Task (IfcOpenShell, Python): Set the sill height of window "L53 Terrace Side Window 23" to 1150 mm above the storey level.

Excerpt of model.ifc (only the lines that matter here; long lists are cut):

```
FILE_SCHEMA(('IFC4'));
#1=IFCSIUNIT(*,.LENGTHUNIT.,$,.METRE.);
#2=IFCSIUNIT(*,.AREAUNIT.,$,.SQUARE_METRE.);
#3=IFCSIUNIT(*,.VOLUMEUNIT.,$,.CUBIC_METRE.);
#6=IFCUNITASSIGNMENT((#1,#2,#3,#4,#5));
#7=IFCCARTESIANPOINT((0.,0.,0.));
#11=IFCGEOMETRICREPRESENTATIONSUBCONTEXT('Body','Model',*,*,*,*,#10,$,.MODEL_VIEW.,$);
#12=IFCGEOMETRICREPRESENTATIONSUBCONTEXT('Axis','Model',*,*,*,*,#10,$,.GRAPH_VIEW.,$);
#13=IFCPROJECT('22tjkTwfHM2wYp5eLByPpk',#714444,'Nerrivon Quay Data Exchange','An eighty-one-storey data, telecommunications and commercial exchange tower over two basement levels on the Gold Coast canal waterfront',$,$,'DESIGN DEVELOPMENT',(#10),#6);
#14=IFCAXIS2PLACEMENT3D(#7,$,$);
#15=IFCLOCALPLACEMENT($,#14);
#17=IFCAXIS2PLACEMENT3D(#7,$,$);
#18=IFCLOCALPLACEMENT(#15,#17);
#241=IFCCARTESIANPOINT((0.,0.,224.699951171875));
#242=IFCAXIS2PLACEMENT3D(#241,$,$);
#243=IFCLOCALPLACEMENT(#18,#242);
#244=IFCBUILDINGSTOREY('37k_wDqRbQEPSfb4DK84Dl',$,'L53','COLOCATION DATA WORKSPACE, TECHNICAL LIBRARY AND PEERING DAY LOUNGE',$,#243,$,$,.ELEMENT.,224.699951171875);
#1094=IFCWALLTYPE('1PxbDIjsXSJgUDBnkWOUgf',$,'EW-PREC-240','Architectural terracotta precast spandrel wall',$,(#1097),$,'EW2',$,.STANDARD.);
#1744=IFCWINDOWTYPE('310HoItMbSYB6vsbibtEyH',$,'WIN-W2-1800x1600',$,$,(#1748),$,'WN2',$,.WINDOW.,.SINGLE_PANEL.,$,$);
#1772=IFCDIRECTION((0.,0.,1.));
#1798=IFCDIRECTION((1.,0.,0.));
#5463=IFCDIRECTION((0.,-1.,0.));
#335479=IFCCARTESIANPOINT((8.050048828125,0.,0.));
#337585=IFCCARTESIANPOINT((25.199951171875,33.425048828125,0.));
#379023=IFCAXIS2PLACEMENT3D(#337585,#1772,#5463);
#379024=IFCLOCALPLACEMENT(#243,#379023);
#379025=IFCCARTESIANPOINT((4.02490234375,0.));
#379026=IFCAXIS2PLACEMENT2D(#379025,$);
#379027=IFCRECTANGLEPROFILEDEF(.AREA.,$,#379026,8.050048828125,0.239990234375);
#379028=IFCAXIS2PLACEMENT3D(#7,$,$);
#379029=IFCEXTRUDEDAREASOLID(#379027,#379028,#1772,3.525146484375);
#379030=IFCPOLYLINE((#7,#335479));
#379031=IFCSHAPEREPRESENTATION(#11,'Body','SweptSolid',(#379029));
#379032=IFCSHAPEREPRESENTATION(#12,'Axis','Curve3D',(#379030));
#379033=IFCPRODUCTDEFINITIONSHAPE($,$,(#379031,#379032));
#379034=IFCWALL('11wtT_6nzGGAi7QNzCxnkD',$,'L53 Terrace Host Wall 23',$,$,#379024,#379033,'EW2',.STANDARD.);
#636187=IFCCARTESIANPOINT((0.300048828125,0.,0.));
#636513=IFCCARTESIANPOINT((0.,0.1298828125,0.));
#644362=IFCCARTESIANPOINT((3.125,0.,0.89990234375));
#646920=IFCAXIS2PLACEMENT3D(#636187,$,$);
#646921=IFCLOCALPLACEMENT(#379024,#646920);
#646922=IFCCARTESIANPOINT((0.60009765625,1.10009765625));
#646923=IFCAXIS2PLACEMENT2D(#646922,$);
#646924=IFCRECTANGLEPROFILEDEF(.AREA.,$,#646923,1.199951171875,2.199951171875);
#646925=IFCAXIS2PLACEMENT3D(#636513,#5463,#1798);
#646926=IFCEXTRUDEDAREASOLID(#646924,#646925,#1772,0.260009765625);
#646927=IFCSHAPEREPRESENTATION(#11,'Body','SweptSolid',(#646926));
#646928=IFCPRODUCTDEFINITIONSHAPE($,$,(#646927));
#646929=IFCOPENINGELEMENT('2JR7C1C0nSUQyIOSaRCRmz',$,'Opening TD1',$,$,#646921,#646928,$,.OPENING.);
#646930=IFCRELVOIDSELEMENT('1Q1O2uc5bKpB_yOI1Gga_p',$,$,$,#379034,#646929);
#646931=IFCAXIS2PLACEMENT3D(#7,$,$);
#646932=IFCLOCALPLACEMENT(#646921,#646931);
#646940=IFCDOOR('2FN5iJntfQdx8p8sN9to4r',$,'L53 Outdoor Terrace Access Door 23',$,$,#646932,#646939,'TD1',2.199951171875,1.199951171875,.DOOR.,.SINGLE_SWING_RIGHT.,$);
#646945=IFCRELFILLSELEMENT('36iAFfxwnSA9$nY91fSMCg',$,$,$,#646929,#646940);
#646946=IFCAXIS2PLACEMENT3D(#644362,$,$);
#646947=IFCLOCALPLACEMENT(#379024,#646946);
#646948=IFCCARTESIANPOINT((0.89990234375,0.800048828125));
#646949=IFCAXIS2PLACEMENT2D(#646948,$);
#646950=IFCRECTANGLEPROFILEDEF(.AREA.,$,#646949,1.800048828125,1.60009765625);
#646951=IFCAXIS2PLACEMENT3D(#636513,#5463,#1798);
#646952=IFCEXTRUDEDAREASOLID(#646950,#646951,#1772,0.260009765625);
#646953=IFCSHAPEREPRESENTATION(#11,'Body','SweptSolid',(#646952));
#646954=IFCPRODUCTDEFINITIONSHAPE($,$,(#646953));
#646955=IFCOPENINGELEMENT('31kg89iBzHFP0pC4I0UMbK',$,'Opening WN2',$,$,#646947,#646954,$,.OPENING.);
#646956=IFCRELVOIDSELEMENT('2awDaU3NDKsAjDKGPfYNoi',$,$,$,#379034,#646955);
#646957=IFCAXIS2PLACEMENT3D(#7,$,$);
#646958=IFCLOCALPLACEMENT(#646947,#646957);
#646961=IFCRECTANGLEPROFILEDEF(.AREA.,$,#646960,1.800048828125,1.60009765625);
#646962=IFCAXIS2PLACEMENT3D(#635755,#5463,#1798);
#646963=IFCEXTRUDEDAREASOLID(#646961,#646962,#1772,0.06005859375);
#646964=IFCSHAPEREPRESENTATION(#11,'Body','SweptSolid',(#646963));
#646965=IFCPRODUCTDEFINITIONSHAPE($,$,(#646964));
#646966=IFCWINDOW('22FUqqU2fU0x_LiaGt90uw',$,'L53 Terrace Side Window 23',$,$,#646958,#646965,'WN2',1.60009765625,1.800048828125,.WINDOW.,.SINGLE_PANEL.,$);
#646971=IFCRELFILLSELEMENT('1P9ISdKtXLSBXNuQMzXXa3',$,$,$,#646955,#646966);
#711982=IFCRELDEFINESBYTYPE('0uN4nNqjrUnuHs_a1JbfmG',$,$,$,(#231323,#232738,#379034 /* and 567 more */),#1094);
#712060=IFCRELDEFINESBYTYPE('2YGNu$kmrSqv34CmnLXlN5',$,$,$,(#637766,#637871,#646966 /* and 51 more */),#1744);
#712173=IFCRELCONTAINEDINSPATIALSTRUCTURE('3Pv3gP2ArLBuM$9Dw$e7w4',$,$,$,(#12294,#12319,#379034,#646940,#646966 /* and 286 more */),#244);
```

```python
import numpy as np
import ifcopenshell
import ifcopenshell.api.geometry
import ifcopenshell.geom
import ifcopenshell.util.element
import ifcopenshell.util.placement
import ifcopenshell.util.shape
import ifcopenshell.util.unit

model = ifcopenshell.open("model.ifc")
unit_scale = ifcopenshell.util.unit.calculate_unit_scale(model)

window = model.by_guid("22FUqqU2fU0x_LiaGt90uw")
opening = window.FillsVoids[0].RelatingOpeningElement
storey = ifcopenshell.util.element.get_container(window, ifc_class="IfcBuildingStorey")
level = ifcopenshell.util.placement.get_local_placement(storey.ObjectPlacement)[2, 3]

# The opening's origin need not be at the sill, so measure its lowest point.
shape = ifcopenshell.geom.create_shape(ifcopenshell.geom.settings(), opening)
bottom = ifcopenshell.util.shape.get_shape_bottom_elevation(shape, shape.geometry) / unit_scale
dz = level + 1.15 / unit_scale - bottom

shift = np.array([0.0, 0.0, dz])
# The window is placed relative to its opening, so it follows when the opening moves.
matrix = ifcopenshell.util.placement.get_local_placement(opening.ObjectPlacement)
matrix[:3, 3] += shift
ifcopenshell.api.geometry.edit_object_placement(
    model, product=opening, matrix=matrix, is_si=False, should_transform_children=True
)

print(f"moved by {dz * unit_scale:+.3f} m")

model.write("model_updated.ifc")
```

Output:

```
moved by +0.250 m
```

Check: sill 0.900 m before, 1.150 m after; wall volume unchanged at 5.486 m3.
